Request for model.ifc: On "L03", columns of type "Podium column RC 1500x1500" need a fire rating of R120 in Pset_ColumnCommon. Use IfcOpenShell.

First a look at what the model holds.

```python
import ifcopenshell
import ifcopenshell.util.element

model = ifcopenshell.open("model.ifc")
print(model.schema)
storey = next(s for s in model.by_type("IfcBuildingStorey") if s.Name == "L03")
columns = [e for e in ifcopenshell.util.element.get_decomposition(storey) if e.is_a("IfcColumn")]
seen = {}
for e in columns:
    element_type = ifcopenshell.util.element.get_type(e)
    key = (element_type.Name if element_type != e and element_type else None, ifcopenshell.util.element.get_pset(e, "Pset_ColumnCommon", "FireRating"))
    seen[key] = seen.get(key, 0) + 1
for (name, value), count in sorted(seen.items(), key=str):
    print(count, "x", name, "|", value)
```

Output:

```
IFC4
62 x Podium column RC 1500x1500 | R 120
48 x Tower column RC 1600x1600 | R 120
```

```python
import ifcopenshell
import ifcopenshell.api.pset
import ifcopenshell.util.element

model = ifcopenshell.open("model.ifc")

storey = next(s for s in model.by_type("IfcBuildingStorey") if s.Name == "L03")
columns = [e for e in ifcopenshell.util.element.get_decomposition(storey) if e.is_a("IfcColumn")]

count = 0
for e in columns:
    element_type = ifcopenshell.util.element.get_type(e)
    if element_type in (None, e) or element_type.Name != "Podium column RC 1500x1500":
        continue
    found = ifcopenshell.util.element.get_pset(e, "Pset_ColumnCommon", should_inherit=False)
    if found:
        pset = model.by_id(found["id"])
        if len(ifcopenshell.util.element.get_elements_by_pset(pset)) > 1:
            pset = ifcopenshell.api.pset.unshare_pset(model, products=[e], pset=pset)[0]
    else:
        pset = ifcopenshell.api.pset.add_pset(model, product=e, name="Pset_ColumnCommon")
    ifcopenshell.api.pset.edit_pset(model, pset=pset, properties={"FireRating": "R120"})
    count += 1

print(count, "columns updated")

model.write("model-out.ifc")
```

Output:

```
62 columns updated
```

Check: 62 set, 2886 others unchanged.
